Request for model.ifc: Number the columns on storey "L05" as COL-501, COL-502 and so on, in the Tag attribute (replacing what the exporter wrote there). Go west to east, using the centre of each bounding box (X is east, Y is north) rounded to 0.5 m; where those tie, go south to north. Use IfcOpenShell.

First a look at what the model holds.

```python
import ifcopenshell
import ifcopenshell.util.element
import ifcopenshell.util.placement

model = ifcopenshell.open("model.ifc")
print(model.schema)
storey = next(s for s in model.by_type("IfcBuildingStorey") if s.Name == "L05")
columns = [e for e in ifcopenshell.util.element.get_decomposition(storey) if e.is_a("IfcColumn")]
for e in sorted(columns, key=lambda e: e.id()):
    origin = ifcopenshell.util.placement.get_local_placement(e.ObjectPlacement)[:3, 3]
    print(e.id(), e.Tag, e.Name, origin.round(2) + 0.0, sep=" | ")
```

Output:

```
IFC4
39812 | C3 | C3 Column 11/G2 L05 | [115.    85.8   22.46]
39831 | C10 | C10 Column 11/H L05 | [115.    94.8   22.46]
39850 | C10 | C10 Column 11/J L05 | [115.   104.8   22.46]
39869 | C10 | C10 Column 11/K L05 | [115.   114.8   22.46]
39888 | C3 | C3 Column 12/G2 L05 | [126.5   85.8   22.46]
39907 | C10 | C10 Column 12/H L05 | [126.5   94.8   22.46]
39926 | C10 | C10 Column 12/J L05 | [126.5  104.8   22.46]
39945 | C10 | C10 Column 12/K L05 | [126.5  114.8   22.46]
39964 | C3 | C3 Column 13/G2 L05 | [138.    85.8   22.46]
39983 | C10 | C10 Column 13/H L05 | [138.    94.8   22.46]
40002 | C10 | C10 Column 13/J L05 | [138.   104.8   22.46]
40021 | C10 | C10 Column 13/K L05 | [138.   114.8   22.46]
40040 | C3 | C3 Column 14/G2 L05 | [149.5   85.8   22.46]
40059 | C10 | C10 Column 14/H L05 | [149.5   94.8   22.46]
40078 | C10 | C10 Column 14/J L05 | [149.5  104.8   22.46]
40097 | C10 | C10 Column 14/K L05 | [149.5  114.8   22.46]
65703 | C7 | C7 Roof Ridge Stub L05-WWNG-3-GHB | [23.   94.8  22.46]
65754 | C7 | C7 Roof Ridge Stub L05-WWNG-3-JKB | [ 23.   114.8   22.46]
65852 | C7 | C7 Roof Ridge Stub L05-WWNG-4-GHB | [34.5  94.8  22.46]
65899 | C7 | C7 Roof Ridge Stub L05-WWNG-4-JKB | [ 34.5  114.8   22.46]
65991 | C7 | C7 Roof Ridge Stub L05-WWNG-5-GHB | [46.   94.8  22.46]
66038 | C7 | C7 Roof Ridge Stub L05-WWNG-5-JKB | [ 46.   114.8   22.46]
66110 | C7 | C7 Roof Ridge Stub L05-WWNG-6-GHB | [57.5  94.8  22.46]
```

```python
import ifcopenshell
import ifcopenshell.geom
import ifcopenshell.util.element
import ifcopenshell.util.shape

model = ifcopenshell.open("model.ifc")
settings = ifcopenshell.geom.settings()
settings.set("use-world-coords", True)


def centre(element):
    shape = ifcopenshell.geom.create_shape(settings, element)
    return ifcopenshell.util.shape.get_bbox_centroid(shape.geometry)


storey = next(s for s in model.by_type("IfcBuildingStorey") if s.Name == "L05")
columns = [e for e in ifcopenshell.util.element.get_decomposition(storey) if e.is_a("IfcColumn")]

# Insertion points can sit at a corner or the storey origin, so sort by the geometry (in metres).
centres = {e: centre(e) for e in columns}
columns.sort(key=lambda e: (round(centres[e][0] / 0.5), centres[e][1]))

for i, e in enumerate(columns, start=1):
    number = f"COL-5{i:02d}"
    e.Tag = number
    print(e.id(), number)

model.write("model_edited.ifc")
```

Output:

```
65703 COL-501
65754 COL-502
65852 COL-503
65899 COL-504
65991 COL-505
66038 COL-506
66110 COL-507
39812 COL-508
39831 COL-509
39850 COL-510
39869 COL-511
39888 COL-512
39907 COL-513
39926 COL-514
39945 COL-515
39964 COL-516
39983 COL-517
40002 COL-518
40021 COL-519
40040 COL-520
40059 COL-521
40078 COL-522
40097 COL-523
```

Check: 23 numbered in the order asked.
